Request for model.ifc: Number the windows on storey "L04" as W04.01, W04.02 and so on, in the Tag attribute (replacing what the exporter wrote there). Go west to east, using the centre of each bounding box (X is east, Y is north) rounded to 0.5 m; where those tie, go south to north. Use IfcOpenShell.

First a look at what the model holds.

```python
import ifcopenshell
import ifcopenshell.util.element
import ifcopenshell.util.placement

model = ifcopenshell.open("model.ifc")
print(model.schema)
storey = next(s for s in model.by_type("IfcBuildingStorey") if s.Name == "L04")
windows = [e for e in ifcopenshell.util.element.get_decomposition(storey) if e.is_a("IfcWindow")]
for e in sorted(windows, key=lambda e: e.id()):
    origin = ifcopenshell.util.placement.get_local_placement(e.ObjectPlacement)[:3, 3]
    print(e.id(), e.Tag, e.Name, origin.round(2) + 0.0, sep=" | ")
```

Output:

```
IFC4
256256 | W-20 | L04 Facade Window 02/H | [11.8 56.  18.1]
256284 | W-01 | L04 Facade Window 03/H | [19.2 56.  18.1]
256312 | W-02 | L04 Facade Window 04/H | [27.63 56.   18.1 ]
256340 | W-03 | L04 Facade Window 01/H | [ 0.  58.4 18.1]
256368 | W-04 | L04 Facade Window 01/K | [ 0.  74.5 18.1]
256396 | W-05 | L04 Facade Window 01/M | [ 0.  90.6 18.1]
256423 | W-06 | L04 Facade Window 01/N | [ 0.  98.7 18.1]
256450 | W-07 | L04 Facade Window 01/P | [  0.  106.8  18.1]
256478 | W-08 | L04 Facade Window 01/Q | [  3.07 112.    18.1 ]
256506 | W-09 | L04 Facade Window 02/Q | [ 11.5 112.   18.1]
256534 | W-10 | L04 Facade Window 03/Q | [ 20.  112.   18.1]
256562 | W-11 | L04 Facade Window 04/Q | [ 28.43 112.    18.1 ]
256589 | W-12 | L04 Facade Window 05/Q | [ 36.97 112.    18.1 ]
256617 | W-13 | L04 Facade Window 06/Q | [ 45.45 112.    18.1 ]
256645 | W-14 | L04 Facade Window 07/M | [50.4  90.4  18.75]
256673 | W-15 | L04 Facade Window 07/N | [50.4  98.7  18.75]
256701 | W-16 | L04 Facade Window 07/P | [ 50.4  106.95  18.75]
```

```python
import ifcopenshell
import ifcopenshell.geom
import ifcopenshell.util.element
import ifcopenshell.util.shape

model = ifcopenshell.open("model.ifc")
settings = ifcopenshell.geom.settings()
settings.set("use-world-coords", True)


def centre(element):
    shape = ifcopenshell.geom.create_shape(settings, element)
    return ifcopenshell.util.shape.get_bbox_centroid(shape.geometry)


storey = next(s for s in model.by_type("IfcBuildingStorey") if s.Name == "L04")
windows = [e for e in ifcopenshell.util.element.get_decomposition(storey) if e.is_a("IfcWindow")]

# Insertion points can sit at a corner or the storey origin, so sort by the geometry (in metres).
centres = {e: centre(e) for e in windows}
windows.sort(key=lambda e: (round(centres[e][0] / 0.5), centres[e][1]))

for i, e in enumerate(windows, start=1):
    number = f"W04.{i:02d}"
    e.Tag = number
    print(e.id(), number)

model.write("model_updated.ifc")
```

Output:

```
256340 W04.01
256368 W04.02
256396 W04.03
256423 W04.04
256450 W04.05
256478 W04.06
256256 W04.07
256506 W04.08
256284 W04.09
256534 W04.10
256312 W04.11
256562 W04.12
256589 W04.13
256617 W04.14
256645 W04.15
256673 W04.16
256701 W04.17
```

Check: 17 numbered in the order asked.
